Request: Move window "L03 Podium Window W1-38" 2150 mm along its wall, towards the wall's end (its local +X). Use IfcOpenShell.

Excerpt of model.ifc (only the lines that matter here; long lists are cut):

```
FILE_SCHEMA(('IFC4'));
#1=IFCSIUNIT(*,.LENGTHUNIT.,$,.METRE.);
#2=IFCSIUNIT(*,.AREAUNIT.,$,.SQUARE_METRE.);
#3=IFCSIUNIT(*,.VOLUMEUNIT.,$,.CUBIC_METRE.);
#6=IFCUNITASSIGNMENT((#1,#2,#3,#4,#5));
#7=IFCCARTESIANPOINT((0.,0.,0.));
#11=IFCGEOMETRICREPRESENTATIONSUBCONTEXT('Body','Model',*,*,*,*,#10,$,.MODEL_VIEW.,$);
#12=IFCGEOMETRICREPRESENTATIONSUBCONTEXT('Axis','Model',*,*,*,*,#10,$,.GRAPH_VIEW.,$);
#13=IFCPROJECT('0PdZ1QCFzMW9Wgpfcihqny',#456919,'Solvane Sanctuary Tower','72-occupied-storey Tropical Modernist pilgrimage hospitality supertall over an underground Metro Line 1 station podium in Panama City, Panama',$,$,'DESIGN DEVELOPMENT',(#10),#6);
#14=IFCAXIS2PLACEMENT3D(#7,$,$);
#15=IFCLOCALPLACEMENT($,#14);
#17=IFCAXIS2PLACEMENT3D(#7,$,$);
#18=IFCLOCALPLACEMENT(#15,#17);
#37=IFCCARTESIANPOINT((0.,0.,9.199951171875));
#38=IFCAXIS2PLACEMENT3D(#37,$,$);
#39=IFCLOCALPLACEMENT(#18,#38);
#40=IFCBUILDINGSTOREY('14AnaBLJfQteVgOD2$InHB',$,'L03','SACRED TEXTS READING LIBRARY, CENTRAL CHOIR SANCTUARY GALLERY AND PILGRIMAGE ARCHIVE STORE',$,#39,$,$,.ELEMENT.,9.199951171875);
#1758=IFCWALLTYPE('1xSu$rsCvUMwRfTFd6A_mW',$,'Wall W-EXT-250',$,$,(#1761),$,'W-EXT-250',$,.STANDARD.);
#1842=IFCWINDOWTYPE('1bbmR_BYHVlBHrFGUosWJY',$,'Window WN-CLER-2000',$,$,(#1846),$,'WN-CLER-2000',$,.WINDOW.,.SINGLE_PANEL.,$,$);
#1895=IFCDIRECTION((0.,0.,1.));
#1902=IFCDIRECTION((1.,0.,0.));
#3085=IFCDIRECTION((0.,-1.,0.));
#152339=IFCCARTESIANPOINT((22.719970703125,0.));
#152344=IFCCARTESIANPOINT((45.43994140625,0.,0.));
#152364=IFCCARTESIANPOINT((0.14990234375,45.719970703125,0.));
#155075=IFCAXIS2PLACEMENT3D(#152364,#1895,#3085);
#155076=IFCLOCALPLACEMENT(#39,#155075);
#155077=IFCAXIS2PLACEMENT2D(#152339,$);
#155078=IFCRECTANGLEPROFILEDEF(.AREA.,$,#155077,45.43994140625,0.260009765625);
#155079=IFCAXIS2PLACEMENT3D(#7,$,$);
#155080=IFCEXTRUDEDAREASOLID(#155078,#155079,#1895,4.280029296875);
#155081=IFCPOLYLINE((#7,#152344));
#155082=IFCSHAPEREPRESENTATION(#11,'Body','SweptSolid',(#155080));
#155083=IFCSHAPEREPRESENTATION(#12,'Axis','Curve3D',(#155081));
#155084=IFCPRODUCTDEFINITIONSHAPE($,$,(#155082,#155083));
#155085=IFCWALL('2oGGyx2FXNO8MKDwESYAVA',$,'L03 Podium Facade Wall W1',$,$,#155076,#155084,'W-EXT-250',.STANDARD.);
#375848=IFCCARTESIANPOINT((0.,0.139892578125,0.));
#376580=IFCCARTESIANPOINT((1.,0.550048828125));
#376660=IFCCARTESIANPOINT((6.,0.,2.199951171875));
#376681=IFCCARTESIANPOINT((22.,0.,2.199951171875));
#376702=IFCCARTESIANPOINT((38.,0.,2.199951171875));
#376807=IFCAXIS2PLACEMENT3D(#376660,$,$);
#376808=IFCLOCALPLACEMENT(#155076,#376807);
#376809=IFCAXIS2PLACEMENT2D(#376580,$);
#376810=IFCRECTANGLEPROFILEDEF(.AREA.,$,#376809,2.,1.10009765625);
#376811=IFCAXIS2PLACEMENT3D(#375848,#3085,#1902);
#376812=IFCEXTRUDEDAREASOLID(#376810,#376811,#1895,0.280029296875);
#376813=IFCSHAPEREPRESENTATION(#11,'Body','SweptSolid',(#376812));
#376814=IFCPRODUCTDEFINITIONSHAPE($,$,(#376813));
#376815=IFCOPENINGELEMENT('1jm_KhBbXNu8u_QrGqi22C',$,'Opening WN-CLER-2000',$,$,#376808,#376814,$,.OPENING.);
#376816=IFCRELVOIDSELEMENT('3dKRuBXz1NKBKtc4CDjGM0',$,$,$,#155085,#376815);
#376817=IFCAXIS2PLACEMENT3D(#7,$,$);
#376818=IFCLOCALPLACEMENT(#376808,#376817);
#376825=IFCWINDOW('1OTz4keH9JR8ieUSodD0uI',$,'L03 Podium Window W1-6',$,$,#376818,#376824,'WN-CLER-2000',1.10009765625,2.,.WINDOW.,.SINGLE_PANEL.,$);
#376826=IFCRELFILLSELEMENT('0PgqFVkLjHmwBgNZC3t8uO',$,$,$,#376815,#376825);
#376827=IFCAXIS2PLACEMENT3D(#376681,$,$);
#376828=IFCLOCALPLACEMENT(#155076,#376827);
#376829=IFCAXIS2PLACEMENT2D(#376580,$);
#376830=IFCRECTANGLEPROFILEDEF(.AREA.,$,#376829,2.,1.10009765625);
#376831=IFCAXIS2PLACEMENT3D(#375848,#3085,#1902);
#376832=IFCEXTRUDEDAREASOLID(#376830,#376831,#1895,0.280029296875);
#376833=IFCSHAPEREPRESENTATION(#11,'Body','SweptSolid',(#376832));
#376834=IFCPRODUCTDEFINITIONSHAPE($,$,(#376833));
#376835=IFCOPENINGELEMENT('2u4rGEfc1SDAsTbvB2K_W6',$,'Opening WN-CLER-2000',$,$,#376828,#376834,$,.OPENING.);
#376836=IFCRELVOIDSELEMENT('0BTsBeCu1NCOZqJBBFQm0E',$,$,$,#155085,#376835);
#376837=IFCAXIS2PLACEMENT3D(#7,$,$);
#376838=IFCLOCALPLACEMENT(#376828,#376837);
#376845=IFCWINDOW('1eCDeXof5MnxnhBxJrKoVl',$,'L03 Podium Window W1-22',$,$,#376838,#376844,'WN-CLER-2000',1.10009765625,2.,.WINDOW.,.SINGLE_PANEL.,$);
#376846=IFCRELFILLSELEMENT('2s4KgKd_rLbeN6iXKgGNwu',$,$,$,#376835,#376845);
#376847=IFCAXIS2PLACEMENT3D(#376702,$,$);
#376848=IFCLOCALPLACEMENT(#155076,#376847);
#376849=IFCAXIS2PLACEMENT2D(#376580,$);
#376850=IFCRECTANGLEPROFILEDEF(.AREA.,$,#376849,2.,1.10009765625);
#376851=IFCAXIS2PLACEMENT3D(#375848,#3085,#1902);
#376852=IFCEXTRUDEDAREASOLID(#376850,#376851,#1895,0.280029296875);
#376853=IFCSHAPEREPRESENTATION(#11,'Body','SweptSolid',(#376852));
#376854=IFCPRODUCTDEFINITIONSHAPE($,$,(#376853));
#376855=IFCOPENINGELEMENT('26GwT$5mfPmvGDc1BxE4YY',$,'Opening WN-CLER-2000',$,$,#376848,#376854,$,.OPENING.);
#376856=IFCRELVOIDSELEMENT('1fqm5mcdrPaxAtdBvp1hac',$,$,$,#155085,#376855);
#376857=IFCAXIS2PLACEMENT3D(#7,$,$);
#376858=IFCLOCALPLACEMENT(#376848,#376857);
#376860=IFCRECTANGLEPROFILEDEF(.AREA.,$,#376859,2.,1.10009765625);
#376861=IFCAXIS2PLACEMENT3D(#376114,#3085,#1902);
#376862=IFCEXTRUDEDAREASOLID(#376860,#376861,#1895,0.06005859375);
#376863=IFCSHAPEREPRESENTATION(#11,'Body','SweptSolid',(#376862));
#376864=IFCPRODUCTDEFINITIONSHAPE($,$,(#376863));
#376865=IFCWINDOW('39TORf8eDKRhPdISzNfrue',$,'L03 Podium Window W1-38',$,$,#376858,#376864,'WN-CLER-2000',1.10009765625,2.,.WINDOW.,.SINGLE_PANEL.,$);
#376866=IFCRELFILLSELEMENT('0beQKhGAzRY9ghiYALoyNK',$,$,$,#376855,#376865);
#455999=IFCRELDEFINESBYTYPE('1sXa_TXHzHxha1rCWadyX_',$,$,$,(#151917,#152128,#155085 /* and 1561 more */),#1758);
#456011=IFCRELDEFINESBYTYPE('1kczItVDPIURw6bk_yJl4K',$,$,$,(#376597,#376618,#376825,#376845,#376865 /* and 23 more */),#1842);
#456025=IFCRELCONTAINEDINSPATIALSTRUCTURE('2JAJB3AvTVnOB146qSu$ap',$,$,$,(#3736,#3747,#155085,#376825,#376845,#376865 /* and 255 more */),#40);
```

```python
import ifcopenshell
import ifcopenshell.api.geometry
import ifcopenshell.util.placement
import ifcopenshell.util.unit

model = ifcopenshell.open("model.ifc")
unit_scale = ifcopenshell.util.unit.calculate_unit_scale(model)

window = model.by_guid("39TORf8eDKRhPdISzNfrue")
opening = window.FillsVoids[0].RelatingOpeningElement
wall = opening.VoidsElements[0].RelatingBuildingElement

wall_matrix = ifcopenshell.util.placement.get_local_placement(wall.ObjectPlacement)
shift = wall_matrix[:3, 0] * 2.15 / unit_scale
before = ifcopenshell.util.placement.get_local_placement(window.ObjectPlacement)[:3, 3].copy()

# The window is placed relative to its opening, so it follows when the opening moves.
matrix = ifcopenshell.util.placement.get_local_placement(opening.ObjectPlacement)
matrix[:3, 3] += shift
ifcopenshell.api.geometry.edit_object_placement(
    model, product=opening, matrix=matrix, is_si=False, should_transform_children=True
)

after = ifcopenshell.util.placement.get_local_placement(window.ObjectPlacement)[:3, 3]
print("window moved by", (after - before).round(3) + 0.0)

model.write("model-out.ifc")
```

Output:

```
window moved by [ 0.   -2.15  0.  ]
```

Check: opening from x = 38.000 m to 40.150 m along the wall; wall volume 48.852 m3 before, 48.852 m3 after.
